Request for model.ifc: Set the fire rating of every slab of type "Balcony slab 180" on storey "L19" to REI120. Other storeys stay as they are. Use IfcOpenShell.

First a look at what the model holds.

```python
import ifcopenshell
import ifcopenshell.util.element

model = ifcopenshell.open("model.ifc")
print(model.schema)
storey = next(s for s in model.by_type("IfcBuildingStorey") if s.Name == "L19")
slabs = [e for e in ifcopenshell.util.element.get_decomposition(storey) if e.is_a("IfcSlab")]
seen = {}
for e in slabs:
    element_type = ifcopenshell.util.element.get_type(e)
    key = (element_type.Name if element_type != e and element_type else None, ifcopenshell.util.element.get_pset(e, "Pset_SlabCommon", "FireRating"))
    seen[key] = seen.get(key, 0) + 1
for (name, value), count in sorted(seen.items(), key=str):
    print(count, "x", name, "|", value)
```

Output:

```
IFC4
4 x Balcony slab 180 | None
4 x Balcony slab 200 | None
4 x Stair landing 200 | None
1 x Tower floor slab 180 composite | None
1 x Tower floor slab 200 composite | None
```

```python
import ifcopenshell
import ifcopenshell.api.pset
import ifcopenshell.util.element

model = ifcopenshell.open("model.ifc")

storey = next(s for s in model.by_type("IfcBuildingStorey") if s.Name == "L19")
slabs = [e for e in ifcopenshell.util.element.get_decomposition(storey) if e.is_a("IfcSlab")]

count = 0
for e in slabs:
    element_type = ifcopenshell.util.element.get_type(e)
    if element_type in (None, e) or element_type.Name != "Balcony slab 180":
        continue
    found = ifcopenshell.util.element.get_pset(e, "Pset_SlabCommon", should_inherit=False)
    if found:
        pset = model.by_id(found["id"])
        if len(ifcopenshell.util.element.get_elements_by_pset(pset)) > 1:
            pset = ifcopenshell.api.pset.unshare_pset(model, products=[e], pset=pset)[0]
    else:
        pset = ifcopenshell.api.pset.add_pset(model, product=e, name="Pset_SlabCommon")
    ifcopenshell.api.pset.edit_pset(model, pset=pset, properties={"FireRating": "REI120"})
    count += 1

print(count, "slabs updated")

model.write("model_rev.ifc")
```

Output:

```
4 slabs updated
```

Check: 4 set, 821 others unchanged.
